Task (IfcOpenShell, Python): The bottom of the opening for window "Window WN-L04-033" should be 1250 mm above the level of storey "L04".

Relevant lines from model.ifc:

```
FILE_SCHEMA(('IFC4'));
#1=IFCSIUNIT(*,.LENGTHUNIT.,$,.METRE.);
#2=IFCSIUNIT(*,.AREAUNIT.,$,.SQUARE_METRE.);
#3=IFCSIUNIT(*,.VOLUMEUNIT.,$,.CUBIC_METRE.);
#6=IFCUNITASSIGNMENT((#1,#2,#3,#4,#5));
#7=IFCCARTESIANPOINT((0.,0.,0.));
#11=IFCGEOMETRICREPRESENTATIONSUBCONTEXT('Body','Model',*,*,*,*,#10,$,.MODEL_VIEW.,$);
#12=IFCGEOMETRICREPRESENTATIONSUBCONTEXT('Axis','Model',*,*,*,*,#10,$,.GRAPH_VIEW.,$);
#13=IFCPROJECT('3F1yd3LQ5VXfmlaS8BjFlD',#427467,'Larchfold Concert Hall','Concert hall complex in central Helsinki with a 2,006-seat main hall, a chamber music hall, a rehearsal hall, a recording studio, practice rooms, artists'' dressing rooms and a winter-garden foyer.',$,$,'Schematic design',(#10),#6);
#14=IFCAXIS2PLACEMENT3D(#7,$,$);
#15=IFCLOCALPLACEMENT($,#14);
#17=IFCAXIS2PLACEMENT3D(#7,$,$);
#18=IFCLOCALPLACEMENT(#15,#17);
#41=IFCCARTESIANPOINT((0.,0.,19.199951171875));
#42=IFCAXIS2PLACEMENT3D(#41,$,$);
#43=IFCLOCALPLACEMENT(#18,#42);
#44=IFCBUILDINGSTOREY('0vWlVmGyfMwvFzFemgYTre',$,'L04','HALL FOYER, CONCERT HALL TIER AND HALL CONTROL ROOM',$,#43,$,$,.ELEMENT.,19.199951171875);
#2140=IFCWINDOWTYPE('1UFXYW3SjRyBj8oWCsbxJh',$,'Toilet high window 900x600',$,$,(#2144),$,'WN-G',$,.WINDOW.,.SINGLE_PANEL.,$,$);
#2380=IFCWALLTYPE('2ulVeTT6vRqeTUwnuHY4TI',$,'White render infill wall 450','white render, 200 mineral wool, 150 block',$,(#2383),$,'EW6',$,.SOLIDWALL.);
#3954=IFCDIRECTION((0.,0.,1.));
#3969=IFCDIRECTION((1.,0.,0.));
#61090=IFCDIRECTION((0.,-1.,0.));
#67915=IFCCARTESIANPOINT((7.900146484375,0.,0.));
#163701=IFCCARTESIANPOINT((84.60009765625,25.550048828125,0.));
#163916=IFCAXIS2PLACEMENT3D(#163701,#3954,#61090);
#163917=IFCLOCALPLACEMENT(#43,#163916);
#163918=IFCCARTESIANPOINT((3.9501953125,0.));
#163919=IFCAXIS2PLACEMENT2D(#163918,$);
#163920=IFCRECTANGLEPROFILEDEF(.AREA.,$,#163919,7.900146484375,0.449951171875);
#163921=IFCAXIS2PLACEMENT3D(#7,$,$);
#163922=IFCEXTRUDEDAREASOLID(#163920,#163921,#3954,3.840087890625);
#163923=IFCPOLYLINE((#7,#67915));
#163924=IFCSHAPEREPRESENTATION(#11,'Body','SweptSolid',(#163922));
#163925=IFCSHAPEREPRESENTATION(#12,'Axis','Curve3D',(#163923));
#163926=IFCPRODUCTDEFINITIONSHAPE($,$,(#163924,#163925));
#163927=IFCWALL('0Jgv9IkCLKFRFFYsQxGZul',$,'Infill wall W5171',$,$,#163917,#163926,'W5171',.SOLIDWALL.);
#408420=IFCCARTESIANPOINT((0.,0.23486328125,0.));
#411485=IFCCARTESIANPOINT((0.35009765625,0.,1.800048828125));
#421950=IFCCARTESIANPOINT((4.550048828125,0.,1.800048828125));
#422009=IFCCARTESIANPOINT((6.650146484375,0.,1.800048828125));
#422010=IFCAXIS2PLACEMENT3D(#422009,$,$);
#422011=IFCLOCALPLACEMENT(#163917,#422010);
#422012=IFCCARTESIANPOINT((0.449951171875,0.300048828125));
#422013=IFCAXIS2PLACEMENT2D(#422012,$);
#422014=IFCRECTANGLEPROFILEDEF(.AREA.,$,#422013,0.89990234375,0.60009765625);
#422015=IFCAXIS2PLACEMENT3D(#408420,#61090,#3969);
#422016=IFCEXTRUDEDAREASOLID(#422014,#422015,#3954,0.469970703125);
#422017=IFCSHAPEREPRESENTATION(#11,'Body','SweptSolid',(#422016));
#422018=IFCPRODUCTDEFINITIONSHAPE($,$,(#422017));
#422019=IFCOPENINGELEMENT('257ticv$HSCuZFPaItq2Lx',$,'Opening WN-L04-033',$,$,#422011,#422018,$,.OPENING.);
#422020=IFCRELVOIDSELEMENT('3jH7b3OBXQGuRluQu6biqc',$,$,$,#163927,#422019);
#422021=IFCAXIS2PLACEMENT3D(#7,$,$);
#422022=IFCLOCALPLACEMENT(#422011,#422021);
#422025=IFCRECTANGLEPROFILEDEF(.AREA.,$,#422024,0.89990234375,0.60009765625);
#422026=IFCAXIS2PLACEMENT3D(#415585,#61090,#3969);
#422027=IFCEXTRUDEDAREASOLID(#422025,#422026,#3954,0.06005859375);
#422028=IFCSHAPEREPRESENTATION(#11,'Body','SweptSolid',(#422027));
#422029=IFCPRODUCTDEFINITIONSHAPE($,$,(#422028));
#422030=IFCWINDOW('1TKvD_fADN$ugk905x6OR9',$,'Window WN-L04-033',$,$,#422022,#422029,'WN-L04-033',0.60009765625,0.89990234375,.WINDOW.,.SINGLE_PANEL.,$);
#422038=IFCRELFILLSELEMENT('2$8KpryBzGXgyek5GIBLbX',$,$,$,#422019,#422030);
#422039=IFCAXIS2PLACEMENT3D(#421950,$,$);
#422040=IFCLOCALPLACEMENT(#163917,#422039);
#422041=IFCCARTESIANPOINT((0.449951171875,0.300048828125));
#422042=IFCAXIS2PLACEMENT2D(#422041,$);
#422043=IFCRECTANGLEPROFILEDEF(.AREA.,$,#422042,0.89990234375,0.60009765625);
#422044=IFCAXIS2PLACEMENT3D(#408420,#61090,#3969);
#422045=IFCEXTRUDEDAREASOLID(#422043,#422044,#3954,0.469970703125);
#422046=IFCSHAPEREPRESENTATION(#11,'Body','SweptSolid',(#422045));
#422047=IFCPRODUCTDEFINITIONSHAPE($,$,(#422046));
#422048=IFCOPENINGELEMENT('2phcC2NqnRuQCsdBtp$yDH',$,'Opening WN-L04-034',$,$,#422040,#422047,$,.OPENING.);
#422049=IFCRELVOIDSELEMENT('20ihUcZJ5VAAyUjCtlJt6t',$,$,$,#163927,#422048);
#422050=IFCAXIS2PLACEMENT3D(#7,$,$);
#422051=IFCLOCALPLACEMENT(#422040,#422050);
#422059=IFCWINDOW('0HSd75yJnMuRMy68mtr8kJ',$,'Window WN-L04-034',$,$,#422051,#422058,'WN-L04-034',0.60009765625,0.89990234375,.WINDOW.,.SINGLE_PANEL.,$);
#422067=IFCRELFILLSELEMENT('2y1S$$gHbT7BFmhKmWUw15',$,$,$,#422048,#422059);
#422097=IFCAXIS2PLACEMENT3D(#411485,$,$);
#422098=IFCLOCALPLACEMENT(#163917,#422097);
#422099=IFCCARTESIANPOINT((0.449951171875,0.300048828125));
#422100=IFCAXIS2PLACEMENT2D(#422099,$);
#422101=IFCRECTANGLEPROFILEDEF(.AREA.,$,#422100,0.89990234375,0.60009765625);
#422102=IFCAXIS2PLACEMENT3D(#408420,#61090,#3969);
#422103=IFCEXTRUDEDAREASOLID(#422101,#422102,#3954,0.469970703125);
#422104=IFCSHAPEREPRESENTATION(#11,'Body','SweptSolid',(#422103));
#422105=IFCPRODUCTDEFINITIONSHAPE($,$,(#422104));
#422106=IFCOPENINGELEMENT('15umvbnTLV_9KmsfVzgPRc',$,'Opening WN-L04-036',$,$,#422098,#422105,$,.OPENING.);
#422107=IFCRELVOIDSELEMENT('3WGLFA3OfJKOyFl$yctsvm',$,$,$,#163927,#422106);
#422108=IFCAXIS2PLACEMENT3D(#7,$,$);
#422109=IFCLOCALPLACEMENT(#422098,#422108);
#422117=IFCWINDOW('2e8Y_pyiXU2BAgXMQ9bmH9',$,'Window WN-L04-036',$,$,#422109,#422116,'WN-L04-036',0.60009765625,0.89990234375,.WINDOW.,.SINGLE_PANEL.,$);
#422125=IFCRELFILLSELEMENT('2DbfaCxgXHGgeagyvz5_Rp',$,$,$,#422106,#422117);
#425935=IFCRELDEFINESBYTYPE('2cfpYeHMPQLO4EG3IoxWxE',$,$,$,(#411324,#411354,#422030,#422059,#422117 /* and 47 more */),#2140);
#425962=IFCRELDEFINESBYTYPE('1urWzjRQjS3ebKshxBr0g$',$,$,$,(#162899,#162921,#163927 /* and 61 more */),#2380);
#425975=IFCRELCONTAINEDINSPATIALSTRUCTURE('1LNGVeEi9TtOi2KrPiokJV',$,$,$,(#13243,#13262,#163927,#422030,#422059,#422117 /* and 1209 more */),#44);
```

```python
import numpy as np
import ifcopenshell
import ifcopenshell.api.geometry
import ifcopenshell.geom
import ifcopenshell.util.element
import ifcopenshell.util.placement
import ifcopenshell.util.shape
import ifcopenshell.util.unit

model = ifcopenshell.open("model.ifc")
unit_scale = ifcopenshell.util.unit.calculate_unit_scale(model)

window = model.by_guid("1TKvD_fADN$ugk905x6OR9")
opening = window.FillsVoids[0].RelatingOpeningElement
storey = ifcopenshell.util.element.get_container(window, ifc_class="IfcBuildingStorey")
level = ifcopenshell.util.placement.get_local_placement(storey.ObjectPlacement)[2, 3]

# The opening's origin need not be at the sill, so measure its lowest point.
shape = ifcopenshell.geom.create_shape(ifcopenshell.geom.settings(), opening)
bottom = ifcopenshell.util.shape.get_shape_bottom_elevation(shape, shape.geometry) / unit_scale
dz = level + 1.25 / unit_scale - bottom

shift = np.array([0.0, 0.0, dz])
# The window is placed relative to its opening, so it follows when the opening moves.
matrix = ifcopenshell.util.placement.get_local_placement(opening.ObjectPlacement)
matrix[:3, 3] += shift
ifcopenshell.api.geometry.edit_object_placement(
    model, product=opening, matrix=matrix, is_si=False, should_transform_children=True
)

print(f"moved by {dz * unit_scale:+.3f} m")

model.write("model_rev.ifc")
```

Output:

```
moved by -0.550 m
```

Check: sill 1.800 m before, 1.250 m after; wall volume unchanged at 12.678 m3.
